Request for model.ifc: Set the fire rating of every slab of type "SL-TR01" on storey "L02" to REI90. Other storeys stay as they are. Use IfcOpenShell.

First a look at what the model holds.

```python
import ifcopenshell
import ifcopenshell.util.element

model = ifcopenshell.open("model.ifc")
print(model.schema)
storey = next(s for s in model.by_type("IfcBuildingStorey") if s.Name == "L02")
slabs = [e for e in ifcopenshell.util.element.get_decomposition(storey) if e.is_a("IfcSlab")]
seen = {}
for e in slabs:
    element_type = ifcopenshell.util.element.get_type(e)
    key = (element_type.Name if element_type != e and element_type else None, ifcopenshell.util.element.get_pset(e, "Pset_SlabCommon", "FireRating"))
    seen[key] = seen.get(key, 0) + 1
for (name, value), count in sorted(seen.items(), key=str):
    print(count, "x", name, "|", value)
```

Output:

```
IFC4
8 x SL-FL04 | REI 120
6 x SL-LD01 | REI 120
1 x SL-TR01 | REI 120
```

```python
import ifcopenshell
import ifcopenshell.api.pset
import ifcopenshell.util.element

model = ifcopenshell.open("model.ifc")

storey = next(s for s in model.by_type("IfcBuildingStorey") if s.Name == "L02")
slabs = [e for e in ifcopenshell.util.element.get_decomposition(storey) if e.is_a("IfcSlab")]

count = 0
for e in slabs:
    element_type = ifcopenshell.util.element.get_type(e)
    if element_type in (None, e) or element_type.Name != "SL-TR01":
        continue
    # add_pset returns the element's existing set when there is one.
    pset = ifcopenshell.api.pset.add_pset(model, product=e, name="Pset_SlabCommon")
    ifcopenshell.api.pset.edit_pset(model, pset=pset, properties={"FireRating": "REI90"})
    count += 1

print(count, "slabs updated")

model.write("model_updated.ifc")
```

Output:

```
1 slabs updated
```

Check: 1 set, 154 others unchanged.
